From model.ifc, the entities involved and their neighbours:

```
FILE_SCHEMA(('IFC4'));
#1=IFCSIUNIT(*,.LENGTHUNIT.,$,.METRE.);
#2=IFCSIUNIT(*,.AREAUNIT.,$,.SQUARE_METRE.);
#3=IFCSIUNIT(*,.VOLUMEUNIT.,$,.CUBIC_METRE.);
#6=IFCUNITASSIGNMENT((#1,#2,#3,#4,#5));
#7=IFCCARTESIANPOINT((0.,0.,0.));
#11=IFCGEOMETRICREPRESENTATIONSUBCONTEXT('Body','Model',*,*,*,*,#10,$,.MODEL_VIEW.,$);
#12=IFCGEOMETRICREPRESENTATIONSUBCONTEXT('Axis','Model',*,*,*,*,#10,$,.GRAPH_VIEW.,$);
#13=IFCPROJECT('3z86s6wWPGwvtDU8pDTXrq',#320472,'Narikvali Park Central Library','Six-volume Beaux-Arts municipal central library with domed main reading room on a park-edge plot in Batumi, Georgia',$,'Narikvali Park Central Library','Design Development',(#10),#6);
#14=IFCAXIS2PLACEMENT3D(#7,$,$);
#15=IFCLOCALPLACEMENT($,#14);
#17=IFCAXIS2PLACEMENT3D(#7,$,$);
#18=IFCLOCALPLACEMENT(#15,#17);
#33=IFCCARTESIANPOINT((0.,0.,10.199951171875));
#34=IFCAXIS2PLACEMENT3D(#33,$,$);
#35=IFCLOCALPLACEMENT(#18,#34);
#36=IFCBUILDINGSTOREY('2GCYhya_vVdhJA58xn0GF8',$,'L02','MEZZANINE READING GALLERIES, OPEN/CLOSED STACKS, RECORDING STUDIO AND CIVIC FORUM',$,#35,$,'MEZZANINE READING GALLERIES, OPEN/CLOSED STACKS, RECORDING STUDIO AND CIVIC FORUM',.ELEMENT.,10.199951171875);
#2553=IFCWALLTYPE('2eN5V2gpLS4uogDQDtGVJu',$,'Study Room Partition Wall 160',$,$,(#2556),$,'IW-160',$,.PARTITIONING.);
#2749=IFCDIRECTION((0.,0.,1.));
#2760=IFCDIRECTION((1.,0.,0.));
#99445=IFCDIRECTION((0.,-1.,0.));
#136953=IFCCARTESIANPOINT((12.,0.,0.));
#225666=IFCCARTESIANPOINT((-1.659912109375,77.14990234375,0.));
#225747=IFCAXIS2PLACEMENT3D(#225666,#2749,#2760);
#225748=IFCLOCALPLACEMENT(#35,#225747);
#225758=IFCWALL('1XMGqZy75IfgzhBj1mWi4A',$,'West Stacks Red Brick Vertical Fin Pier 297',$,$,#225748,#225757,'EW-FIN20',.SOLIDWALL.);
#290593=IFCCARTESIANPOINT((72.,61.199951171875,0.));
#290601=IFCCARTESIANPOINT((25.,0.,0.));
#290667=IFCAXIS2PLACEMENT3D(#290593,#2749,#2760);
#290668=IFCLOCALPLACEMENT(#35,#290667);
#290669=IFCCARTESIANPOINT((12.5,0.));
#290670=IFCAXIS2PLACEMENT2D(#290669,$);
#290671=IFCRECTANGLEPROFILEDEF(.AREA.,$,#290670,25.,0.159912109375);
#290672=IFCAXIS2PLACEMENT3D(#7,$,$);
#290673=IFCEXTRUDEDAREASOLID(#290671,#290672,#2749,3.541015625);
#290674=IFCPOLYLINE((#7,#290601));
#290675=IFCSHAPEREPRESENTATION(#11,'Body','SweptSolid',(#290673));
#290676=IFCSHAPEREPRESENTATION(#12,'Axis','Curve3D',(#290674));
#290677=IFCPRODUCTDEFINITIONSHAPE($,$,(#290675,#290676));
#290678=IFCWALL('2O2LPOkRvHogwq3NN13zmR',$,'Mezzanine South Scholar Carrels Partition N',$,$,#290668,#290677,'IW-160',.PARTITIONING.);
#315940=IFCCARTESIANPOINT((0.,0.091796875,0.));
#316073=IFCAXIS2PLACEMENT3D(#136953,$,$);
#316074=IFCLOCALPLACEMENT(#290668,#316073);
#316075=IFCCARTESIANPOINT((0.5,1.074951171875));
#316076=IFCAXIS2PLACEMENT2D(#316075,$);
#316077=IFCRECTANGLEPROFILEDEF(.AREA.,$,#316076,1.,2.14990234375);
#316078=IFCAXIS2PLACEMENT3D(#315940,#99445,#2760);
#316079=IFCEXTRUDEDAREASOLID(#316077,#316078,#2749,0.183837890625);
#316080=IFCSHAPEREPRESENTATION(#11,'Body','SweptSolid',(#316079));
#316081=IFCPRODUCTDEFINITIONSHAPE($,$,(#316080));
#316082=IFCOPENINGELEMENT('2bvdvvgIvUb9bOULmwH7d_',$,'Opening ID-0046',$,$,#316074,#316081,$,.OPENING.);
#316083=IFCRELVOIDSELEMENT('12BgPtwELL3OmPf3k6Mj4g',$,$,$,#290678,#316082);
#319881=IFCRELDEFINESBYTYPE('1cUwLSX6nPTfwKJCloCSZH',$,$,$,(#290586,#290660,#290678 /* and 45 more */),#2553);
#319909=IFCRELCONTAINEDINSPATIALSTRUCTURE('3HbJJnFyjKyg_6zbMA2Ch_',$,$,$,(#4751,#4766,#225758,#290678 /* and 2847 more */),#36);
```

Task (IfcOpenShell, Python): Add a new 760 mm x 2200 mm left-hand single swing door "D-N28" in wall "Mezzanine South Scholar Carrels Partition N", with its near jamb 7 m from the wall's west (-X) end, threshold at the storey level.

```python
import numpy as np
import ifcopenshell
import ifcopenshell.api.feature
import ifcopenshell.api.geometry
import ifcopenshell.api.root
import ifcopenshell.api.spatial
import ifcopenshell.geom
import ifcopenshell.util.element
import ifcopenshell.util.placement
import ifcopenshell.util.representation
import ifcopenshell.util.shape
import ifcopenshell.util.unit

model = ifcopenshell.open("model.ifc")
unit_scale = ifcopenshell.util.unit.calculate_unit_scale(model)
settings = ifcopenshell.geom.settings()


def volume(element):
    """Net volume in cubic metres, openings subtracted."""
    shape = ifcopenshell.geom.create_shape(settings, element)
    return ifcopenshell.util.shape.get_volume(shape.geometry)


wall = model.by_guid("2O2LPOkRvHogwq3NN13zmR")
storey = ifcopenshell.util.element.get_container(wall, ifc_class="IfcBuildingStorey")
context = ifcopenshell.util.representation.get_context(model, "Model", "Body", "MODEL_VIEW")
before = volume(wall)

width, height, from_end, sill = 0.76, 2.2, 7, 0.0  # metres

# The wall runs along its own X axis, and the end named is its -X end.
wall_shape = ifcopenshell.geom.create_shape(settings, wall)
x, y, z = ifcopenshell.util.shape.get_vertices(wall_shape.geometry).T
start = x.min() + from_end
face, thickness = float(y.min()), float(y.max() - y.min())
wall_matrix = ifcopenshell.util.placement.get_local_placement(wall.ObjectPlacement)
level = ifcopenshell.util.placement.get_local_placement(storey.ObjectPlacement)[2, 3]


def in_wall(x, y):
    """Placement at x, y metres in the wall's axes, at sill height."""
    matrix = wall_matrix.copy()
    matrix[:, 3] = wall_matrix @ np.array([x / unit_scale, y / unit_scale, 0.0, 1.0])
    matrix[2, 3] = level + sill / unit_scale
    return matrix


# Opening: a box that overshoots both wall faces by 50 mm.
opening = ifcopenshell.api.root.create_entity(model, ifc_class="IfcOpeningElement", predefined_type="OPENING")
box = ifcopenshell.api.geometry.add_wall_representation(
    model, context=context, length=width, height=height, thickness=thickness + 0.1
)
ifcopenshell.api.geometry.assign_representation(model, product=opening, representation=box)
ifcopenshell.api.geometry.edit_object_placement(model, product=opening, matrix=in_wall(start, face - 0.05), is_si=False)
ifcopenshell.api.feature.add_feature(model, feature=opening, element=wall)

door = ifcopenshell.api.root.create_entity(model, ifc_class="IfcDoor", name="D-N28", predefined_type="DOOR")
door.OverallWidth, door.OverallHeight = width / unit_scale, height / unit_scale
door.OperationType = "SINGLE_SWING_LEFT"
body = ifcopenshell.api.geometry.add_door_representation(
    model,
    context=context,
    overall_width=door.OverallWidth,
    overall_height=door.OverallHeight,
    operation_type="SINGLE_SWING_LEFT",
    lining_properties={"LiningDepth": thickness / unit_scale, "ThresholdDepth": thickness / unit_scale},
)
ifcopenshell.api.geometry.assign_representation(model, product=door, representation=body)
ifcopenshell.api.spatial.assign_container(model, products=[door], relating_structure=storey)
ifcopenshell.api.feature.add_filling(model, opening=opening, element=door)

# The lining spans the wall, so the door starts at the wall face.
ifcopenshell.api.geometry.edit_object_placement(model, product=door, matrix=in_wall(start, face), is_si=False)

after = volume(wall)

print(f"wall volume {before:.3f} -> {after:.3f} m3")

model.write("model_edited.ifc")
```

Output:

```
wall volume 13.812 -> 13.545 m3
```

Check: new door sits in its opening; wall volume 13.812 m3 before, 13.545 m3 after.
